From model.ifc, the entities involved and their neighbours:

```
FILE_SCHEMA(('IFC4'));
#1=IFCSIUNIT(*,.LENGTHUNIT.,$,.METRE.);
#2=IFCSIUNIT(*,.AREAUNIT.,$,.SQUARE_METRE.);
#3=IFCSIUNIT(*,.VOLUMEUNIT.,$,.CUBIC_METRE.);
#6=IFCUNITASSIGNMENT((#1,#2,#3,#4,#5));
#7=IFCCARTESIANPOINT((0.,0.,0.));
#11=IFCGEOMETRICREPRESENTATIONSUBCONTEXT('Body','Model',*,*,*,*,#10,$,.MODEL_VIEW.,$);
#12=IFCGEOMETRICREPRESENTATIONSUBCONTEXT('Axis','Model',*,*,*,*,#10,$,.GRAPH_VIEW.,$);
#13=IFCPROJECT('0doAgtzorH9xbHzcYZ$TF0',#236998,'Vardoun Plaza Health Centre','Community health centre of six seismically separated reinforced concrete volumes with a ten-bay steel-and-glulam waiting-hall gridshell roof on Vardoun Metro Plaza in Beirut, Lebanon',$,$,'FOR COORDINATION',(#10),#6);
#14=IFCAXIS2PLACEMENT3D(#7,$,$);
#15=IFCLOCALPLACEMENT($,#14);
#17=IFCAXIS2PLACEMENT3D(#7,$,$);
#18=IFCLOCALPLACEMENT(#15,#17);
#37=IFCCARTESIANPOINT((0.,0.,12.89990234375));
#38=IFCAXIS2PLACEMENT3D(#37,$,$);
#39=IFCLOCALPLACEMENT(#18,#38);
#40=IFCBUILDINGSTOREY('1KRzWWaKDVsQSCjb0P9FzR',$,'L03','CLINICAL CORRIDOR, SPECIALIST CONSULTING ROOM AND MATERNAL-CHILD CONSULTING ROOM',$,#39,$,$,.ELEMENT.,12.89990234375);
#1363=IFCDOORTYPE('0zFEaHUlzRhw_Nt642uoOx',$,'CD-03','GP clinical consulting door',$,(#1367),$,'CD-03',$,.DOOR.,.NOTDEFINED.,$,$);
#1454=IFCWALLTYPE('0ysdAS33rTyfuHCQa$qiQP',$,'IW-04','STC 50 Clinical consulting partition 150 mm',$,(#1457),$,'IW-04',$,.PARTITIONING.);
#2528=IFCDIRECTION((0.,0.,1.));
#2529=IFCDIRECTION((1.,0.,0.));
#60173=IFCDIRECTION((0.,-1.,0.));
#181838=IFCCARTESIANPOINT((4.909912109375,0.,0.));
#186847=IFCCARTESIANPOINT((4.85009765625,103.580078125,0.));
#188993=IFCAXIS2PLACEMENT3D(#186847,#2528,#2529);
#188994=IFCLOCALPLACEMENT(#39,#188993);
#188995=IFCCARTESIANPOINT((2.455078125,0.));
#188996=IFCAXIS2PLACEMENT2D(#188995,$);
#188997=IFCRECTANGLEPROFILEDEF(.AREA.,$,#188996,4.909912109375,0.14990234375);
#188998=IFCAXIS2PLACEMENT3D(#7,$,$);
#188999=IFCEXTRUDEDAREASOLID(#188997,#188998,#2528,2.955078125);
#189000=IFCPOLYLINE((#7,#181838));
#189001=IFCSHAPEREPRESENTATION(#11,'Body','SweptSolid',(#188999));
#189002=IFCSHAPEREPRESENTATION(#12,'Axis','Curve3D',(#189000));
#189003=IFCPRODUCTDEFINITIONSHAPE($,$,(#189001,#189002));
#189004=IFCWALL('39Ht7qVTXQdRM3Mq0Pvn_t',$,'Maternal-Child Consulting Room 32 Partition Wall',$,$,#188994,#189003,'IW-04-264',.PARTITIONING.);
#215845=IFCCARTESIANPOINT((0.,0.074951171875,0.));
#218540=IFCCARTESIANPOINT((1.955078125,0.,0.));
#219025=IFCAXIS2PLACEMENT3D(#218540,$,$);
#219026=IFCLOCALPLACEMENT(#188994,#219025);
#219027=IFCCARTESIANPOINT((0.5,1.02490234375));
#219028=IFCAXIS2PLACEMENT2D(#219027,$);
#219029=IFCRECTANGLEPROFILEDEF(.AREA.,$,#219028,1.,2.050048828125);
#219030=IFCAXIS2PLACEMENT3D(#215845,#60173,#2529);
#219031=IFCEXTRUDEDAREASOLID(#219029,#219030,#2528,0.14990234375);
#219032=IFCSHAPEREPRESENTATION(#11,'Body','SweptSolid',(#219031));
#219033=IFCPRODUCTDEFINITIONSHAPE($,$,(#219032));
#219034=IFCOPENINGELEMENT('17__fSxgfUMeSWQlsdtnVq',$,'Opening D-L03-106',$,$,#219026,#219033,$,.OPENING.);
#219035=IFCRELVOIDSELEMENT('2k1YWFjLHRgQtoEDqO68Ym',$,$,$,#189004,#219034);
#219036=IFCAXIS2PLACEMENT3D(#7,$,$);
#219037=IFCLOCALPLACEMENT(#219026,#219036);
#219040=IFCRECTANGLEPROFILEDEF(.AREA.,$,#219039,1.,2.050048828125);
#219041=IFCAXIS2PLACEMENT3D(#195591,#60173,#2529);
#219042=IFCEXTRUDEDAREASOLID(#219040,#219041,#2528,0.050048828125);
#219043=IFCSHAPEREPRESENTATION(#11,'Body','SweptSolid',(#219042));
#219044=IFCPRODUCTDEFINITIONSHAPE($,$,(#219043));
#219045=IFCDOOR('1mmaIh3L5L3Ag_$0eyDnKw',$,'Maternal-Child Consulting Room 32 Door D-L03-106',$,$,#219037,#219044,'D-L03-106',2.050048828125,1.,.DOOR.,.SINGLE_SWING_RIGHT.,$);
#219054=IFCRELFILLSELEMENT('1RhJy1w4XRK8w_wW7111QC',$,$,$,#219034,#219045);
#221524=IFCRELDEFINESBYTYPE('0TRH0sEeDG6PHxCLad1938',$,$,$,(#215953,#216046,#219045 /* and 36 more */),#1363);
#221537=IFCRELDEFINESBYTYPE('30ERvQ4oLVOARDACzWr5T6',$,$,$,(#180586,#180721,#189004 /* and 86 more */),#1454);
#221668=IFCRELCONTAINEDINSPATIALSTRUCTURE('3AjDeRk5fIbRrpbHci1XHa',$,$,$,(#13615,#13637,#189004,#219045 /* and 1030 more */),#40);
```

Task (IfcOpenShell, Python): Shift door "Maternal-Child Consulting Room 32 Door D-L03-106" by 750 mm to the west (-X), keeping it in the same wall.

```python
import ifcopenshell
import ifcopenshell.api.geometry
import ifcopenshell.util.placement
import ifcopenshell.util.unit

model = ifcopenshell.open("model.ifc")
unit_scale = ifcopenshell.util.unit.calculate_unit_scale(model)

door = model.by_guid("1mmaIh3L5L3Ag_$0eyDnKw")
opening = door.FillsVoids[0].RelatingOpeningElement
wall = opening.VoidsElements[0].RelatingBuildingElement

wall_matrix = ifcopenshell.util.placement.get_local_placement(wall.ObjectPlacement)
shift = wall_matrix[:3, 0] * -0.75 / unit_scale
before = ifcopenshell.util.placement.get_local_placement(door.ObjectPlacement)[:3, 3].copy()

# The door is placed relative to its opening, so it follows when the opening moves.
matrix = ifcopenshell.util.placement.get_local_placement(opening.ObjectPlacement)
matrix[:3, 3] += shift
ifcopenshell.api.geometry.edit_object_placement(
    model, product=opening, matrix=matrix, is_si=False, should_transform_children=True
)

after = ifcopenshell.util.placement.get_local_placement(door.ObjectPlacement)[:3, 3]
print("door moved by", (after - before).round(3) + 0.0)

model.write("model_edited.ifc")
```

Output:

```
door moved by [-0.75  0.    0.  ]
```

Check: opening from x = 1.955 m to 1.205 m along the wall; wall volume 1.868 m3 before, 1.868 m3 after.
